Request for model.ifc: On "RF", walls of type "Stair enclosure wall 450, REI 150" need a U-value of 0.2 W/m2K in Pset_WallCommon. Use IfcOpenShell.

First a look at what the model holds.

```python
import ifcopenshell
import ifcopenshell.util.element

model = ifcopenshell.open("model.ifc")
print(model.schema)
storey = next(s for s in model.by_type("IfcBuildingStorey") if s.Name == "RF")
walls = [e for e in ifcopenshell.util.element.get_decomposition(storey) if e.is_a("IfcWall")]
seen = {}
for e in walls:
    element_type = ifcopenshell.util.element.get_type(e)
    key = (element_type.Name if element_type != e and element_type else None, ifcopenshell.util.element.get_pset(e, "Pset_WallCommon", "ThermalTransmittance"))
    seen[key] = seen.get(key, 0) + 1
for (name, value), count in sorted(seen.items(), key=str):
    print(count, "x", name, "|", value)
```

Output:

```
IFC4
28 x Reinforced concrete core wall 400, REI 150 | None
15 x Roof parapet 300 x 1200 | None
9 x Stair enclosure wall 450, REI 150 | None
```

```python
import ifcopenshell
import ifcopenshell.api.pset
import ifcopenshell.util.element

model = ifcopenshell.open("model.ifc")

storey = next(s for s in model.by_type("IfcBuildingStorey") if s.Name == "RF")
walls = [e for e in ifcopenshell.util.element.get_decomposition(storey) if e.is_a("IfcWall")]

count = 0
for e in walls:
    element_type = ifcopenshell.util.element.get_type(e)
    if element_type in (None, e) or element_type.Name != "Stair enclosure wall 450, REI 150":
        continue
    # add_pset returns the element's existing set when there is one.
    pset = ifcopenshell.api.pset.add_pset(model, product=e, name="Pset_WallCommon")
    ifcopenshell.api.pset.edit_pset(model, pset=pset, properties={"ThermalTransmittance": 0.2})
    count += 1

print(count, "walls updated")

model.write("model_edited.ifc")
```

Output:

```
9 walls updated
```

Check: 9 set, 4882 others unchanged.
